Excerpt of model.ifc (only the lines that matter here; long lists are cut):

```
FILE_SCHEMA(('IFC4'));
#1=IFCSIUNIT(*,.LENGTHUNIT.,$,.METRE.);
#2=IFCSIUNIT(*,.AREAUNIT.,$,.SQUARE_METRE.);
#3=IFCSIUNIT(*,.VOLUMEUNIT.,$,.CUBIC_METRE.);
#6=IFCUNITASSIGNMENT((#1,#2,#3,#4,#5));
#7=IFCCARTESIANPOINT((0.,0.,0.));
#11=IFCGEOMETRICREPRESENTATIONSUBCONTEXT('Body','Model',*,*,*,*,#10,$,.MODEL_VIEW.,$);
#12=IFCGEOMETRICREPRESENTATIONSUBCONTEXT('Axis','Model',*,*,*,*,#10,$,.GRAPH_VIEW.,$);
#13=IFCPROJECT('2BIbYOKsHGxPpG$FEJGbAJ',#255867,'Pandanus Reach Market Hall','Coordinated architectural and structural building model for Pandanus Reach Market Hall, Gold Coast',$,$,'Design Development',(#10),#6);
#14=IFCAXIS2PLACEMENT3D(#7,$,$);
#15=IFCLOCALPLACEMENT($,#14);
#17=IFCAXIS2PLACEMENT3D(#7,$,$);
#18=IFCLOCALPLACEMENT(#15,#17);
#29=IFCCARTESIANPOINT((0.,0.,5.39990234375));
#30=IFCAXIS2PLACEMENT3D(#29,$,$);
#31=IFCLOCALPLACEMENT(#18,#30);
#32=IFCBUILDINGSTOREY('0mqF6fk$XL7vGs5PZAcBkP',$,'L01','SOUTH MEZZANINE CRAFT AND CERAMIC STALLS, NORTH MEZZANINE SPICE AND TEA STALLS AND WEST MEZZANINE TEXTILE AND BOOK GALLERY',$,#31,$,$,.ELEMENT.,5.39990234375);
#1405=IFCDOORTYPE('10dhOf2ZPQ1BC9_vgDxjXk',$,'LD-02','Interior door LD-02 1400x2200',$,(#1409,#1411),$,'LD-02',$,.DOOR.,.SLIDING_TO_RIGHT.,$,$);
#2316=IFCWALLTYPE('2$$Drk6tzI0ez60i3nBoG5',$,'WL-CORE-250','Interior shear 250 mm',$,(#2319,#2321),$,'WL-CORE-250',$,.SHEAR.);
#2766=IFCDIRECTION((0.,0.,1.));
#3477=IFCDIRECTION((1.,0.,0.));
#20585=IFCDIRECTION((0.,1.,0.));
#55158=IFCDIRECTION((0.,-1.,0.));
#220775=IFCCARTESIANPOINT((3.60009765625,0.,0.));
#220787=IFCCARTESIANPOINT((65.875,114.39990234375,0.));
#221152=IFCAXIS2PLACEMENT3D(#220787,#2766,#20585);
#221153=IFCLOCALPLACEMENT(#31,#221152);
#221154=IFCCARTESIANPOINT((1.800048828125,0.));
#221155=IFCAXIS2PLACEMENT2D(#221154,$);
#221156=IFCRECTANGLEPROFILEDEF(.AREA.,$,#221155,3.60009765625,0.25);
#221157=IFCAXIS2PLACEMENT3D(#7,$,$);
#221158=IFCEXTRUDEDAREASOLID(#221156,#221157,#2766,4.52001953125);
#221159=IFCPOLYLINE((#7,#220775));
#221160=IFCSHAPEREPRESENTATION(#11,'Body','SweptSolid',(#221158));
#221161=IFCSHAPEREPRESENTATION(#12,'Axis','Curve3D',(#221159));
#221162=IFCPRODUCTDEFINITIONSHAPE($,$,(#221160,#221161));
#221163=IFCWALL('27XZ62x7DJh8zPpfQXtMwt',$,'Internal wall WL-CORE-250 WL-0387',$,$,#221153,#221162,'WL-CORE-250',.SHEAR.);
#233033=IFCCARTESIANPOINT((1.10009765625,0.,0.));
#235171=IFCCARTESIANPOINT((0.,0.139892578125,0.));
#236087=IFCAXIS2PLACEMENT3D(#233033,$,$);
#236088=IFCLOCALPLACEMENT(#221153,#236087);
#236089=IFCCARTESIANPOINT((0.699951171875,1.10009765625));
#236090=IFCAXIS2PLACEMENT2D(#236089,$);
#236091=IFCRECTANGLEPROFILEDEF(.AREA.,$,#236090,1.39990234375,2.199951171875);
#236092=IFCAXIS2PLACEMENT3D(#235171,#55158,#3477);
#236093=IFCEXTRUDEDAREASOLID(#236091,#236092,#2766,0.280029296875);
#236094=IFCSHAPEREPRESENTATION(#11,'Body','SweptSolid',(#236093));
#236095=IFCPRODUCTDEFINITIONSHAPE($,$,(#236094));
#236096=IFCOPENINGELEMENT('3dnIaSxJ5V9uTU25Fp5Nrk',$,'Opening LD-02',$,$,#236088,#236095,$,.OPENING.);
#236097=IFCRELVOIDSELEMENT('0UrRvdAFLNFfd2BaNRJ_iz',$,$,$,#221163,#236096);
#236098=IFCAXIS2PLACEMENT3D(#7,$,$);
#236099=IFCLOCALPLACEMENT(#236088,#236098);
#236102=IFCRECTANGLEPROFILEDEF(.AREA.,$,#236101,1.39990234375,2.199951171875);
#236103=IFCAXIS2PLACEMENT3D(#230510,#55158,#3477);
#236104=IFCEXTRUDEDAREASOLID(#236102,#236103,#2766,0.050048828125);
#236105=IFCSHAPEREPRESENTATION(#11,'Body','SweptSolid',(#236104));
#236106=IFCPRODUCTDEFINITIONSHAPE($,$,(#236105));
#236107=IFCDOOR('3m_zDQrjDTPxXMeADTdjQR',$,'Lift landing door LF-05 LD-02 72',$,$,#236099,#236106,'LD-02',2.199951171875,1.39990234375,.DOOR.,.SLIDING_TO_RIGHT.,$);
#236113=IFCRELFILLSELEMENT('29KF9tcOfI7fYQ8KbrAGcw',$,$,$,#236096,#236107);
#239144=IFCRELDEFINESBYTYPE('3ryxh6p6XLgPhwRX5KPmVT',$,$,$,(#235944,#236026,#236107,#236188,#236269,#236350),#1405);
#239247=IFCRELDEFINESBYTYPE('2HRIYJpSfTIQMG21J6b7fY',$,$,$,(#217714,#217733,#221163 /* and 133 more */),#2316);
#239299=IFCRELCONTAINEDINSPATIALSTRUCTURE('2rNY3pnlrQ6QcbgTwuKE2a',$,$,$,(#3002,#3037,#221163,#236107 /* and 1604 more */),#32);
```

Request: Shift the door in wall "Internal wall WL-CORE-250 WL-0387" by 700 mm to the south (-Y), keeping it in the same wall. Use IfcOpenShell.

```python
import ifcopenshell
import ifcopenshell.api.geometry
import ifcopenshell.util.placement
import ifcopenshell.util.unit

model = ifcopenshell.open("model.ifc")
unit_scale = ifcopenshell.util.unit.calculate_unit_scale(model)

door = model.by_id(236107)
opening = door.FillsVoids[0].RelatingOpeningElement
wall = opening.VoidsElements[0].RelatingBuildingElement

wall_matrix = ifcopenshell.util.placement.get_local_placement(wall.ObjectPlacement)
shift = wall_matrix[:3, 0] * -0.7 / unit_scale
before = ifcopenshell.util.placement.get_local_placement(door.ObjectPlacement)[:3, 3].copy()

# The door is placed relative to its opening, so it follows when the opening moves.
matrix = ifcopenshell.util.placement.get_local_placement(opening.ObjectPlacement)
matrix[:3, 3] += shift
ifcopenshell.api.geometry.edit_object_placement(
    model, product=opening, matrix=matrix, is_si=False, should_transform_children=True
)

after = ifcopenshell.util.placement.get_local_placement(door.ObjectPlacement)[:3, 3]
print("door moved by", (after - before).round(3) + 0.0)

model.write("model-out.ifc")
```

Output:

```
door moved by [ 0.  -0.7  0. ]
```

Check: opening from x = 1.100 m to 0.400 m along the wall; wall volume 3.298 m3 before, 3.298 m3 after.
